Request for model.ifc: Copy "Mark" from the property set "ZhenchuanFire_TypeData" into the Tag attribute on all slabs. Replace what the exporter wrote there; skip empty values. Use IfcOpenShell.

First a look at what the model holds.

```python
import ifcopenshell
import ifcopenshell.util.element

model = ifcopenshell.open("model.ifc")
print(model.schema)
slabs = model.by_type("IfcSlab")
print(len(slabs), "slabs")
for e in slabs[:8]:
    source = ifcopenshell.util.element.get_pset(e, "ZhenchuanFire_TypeData", "Mark")
    target = e.Tag
    print(e.id(), repr(source), repr(target), sep=" | ")
```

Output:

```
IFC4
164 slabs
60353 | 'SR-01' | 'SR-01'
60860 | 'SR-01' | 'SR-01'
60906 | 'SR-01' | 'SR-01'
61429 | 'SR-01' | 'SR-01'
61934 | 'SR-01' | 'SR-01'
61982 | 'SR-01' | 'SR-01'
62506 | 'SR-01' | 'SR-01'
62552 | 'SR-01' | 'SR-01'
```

```python
import ifcopenshell
import ifcopenshell.util.element

model = ifcopenshell.open("model.ifc")

count = 0
for e in model.by_type("IfcSlab"):
    value = ifcopenshell.util.element.get_pset(e, "ZhenchuanFire_TypeData", "Mark")
    current = e.Tag
    if not value or not value.strip() or current == value:
        continue
    e.Tag = value
    count += 1

print(count, "slabs updated")

model.write("model_updated.ifc")
```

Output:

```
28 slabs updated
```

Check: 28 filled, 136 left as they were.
